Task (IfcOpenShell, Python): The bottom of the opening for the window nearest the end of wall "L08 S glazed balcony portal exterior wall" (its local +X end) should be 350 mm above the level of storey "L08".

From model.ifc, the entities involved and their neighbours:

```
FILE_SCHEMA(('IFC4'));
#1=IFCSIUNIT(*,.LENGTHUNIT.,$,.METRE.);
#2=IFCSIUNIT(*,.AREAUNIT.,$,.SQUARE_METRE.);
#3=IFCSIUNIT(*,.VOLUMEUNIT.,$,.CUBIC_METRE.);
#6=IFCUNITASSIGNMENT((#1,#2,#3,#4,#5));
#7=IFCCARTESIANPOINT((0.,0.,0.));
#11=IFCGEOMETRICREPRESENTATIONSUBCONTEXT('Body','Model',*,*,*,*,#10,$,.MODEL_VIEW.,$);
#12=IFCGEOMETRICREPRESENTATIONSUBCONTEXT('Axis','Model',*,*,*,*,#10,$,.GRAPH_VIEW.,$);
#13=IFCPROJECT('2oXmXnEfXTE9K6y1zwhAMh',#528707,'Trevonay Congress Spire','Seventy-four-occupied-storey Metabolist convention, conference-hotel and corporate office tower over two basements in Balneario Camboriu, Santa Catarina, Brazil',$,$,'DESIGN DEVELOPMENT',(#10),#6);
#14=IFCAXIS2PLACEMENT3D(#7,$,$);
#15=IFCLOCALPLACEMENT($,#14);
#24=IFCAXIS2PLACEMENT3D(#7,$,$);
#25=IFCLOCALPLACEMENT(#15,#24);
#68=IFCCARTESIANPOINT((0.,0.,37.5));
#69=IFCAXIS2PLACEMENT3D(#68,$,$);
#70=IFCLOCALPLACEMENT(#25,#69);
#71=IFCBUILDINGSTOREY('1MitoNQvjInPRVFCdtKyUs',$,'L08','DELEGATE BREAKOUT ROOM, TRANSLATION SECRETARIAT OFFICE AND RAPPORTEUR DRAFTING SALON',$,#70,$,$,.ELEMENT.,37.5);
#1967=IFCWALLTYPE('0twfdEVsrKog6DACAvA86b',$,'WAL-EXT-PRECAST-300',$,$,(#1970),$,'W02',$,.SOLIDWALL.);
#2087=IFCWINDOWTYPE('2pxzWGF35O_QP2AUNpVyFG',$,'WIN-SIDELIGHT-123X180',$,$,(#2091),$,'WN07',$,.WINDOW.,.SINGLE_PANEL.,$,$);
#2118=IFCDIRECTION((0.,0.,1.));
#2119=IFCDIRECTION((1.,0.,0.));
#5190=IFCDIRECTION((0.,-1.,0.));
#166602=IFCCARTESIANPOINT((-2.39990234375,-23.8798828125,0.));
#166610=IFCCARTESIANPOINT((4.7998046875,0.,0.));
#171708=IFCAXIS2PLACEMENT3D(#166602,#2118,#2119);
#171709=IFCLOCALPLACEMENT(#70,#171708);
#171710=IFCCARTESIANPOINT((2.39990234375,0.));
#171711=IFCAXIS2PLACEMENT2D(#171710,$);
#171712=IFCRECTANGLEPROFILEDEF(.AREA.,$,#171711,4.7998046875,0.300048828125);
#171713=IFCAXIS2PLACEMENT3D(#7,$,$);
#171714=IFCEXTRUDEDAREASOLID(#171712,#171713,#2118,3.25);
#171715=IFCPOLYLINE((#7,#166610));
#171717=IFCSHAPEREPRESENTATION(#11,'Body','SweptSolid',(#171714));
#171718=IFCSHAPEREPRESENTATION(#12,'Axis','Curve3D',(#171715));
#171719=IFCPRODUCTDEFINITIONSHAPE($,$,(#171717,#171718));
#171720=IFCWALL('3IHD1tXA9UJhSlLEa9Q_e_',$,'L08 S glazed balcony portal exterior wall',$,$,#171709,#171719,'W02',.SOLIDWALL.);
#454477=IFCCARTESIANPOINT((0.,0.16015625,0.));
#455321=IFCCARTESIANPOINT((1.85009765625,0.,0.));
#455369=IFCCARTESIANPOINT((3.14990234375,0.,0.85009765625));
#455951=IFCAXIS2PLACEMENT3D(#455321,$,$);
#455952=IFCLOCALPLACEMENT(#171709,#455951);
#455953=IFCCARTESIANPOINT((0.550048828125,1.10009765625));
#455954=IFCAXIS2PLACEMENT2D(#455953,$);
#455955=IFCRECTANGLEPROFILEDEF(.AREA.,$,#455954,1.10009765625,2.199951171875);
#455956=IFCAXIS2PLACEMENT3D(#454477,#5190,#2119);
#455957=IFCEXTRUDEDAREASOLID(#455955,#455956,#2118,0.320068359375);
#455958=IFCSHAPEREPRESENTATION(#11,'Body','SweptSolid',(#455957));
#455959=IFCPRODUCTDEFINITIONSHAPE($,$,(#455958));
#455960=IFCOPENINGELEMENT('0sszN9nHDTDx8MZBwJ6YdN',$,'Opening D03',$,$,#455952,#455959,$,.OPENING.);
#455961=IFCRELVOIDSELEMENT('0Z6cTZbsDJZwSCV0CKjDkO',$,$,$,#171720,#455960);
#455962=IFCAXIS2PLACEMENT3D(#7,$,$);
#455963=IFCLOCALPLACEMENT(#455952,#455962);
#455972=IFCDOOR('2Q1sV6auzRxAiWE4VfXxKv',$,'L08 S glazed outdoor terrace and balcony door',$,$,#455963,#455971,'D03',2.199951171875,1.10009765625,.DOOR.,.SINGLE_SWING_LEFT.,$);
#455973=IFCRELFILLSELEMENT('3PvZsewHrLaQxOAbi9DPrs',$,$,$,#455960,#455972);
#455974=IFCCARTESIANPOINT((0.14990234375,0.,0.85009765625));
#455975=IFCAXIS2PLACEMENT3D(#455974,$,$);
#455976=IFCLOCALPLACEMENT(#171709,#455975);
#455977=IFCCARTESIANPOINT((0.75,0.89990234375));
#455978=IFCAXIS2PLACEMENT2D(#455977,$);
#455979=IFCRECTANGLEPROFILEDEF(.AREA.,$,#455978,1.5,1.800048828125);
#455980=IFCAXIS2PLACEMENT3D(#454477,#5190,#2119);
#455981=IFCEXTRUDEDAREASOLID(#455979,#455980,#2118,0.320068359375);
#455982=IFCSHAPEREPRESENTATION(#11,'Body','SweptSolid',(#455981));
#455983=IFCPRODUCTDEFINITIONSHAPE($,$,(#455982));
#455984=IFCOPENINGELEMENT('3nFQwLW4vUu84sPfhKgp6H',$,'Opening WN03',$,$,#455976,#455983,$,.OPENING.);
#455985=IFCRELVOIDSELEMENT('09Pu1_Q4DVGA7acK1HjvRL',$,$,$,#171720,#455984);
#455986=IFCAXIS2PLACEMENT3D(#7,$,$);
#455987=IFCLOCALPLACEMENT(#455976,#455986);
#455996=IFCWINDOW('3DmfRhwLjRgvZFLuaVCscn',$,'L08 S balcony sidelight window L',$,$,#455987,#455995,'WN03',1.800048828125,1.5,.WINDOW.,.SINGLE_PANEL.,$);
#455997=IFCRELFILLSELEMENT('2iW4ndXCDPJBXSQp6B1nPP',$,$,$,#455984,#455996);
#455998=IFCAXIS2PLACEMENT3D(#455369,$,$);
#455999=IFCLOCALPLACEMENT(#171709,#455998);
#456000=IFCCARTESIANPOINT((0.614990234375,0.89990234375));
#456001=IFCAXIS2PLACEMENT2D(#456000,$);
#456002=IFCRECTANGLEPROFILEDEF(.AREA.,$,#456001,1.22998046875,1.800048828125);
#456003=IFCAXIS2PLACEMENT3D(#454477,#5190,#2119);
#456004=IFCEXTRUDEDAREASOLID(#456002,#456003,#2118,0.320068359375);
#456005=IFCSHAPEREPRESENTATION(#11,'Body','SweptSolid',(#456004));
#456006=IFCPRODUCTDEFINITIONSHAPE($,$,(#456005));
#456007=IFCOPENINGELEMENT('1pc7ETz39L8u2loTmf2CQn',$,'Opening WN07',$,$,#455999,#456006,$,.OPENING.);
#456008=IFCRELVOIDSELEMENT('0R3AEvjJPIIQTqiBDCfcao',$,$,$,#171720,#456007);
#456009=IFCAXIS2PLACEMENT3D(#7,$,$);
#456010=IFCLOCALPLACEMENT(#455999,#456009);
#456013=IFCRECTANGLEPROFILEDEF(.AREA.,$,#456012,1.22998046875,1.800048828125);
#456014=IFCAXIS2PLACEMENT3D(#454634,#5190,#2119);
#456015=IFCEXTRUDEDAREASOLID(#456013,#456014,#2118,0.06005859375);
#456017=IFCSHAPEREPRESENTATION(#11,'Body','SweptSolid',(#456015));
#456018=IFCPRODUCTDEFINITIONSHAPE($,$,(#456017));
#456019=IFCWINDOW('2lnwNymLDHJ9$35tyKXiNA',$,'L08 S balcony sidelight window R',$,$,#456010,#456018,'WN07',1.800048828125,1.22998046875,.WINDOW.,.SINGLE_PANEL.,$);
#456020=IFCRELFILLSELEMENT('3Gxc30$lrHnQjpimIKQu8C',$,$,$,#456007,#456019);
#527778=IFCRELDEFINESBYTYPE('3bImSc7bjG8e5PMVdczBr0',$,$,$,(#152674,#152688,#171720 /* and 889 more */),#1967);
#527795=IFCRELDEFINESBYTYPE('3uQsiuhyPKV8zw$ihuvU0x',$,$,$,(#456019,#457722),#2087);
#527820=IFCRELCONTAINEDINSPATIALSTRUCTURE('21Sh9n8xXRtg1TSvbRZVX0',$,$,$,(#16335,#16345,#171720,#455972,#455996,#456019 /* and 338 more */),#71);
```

```python
import numpy as np
import ifcopenshell
import ifcopenshell.api.geometry
import ifcopenshell.geom
import ifcopenshell.util.element
import ifcopenshell.util.placement
import ifcopenshell.util.shape
import ifcopenshell.util.unit

model = ifcopenshell.open("model.ifc")
unit_scale = ifcopenshell.util.unit.calculate_unit_scale(model)

window = model.by_guid("2lnwNymLDHJ9$35tyKXiNA")
opening = window.FillsVoids[0].RelatingOpeningElement
storey = ifcopenshell.util.element.get_container(window, ifc_class="IfcBuildingStorey")
level = ifcopenshell.util.placement.get_local_placement(storey.ObjectPlacement)[2, 3]

# The opening's origin need not be at the sill, so measure its lowest point.
shape = ifcopenshell.geom.create_shape(ifcopenshell.geom.settings(), opening)
bottom = ifcopenshell.util.shape.get_shape_bottom_elevation(shape, shape.geometry) / unit_scale
dz = level + 0.35 / unit_scale - bottom

shift = np.array([0.0, 0.0, dz])
# The window is placed relative to its opening, so it follows when the opening moves.
matrix = ifcopenshell.util.placement.get_local_placement(opening.ObjectPlacement)
matrix[:3, 3] += shift
ifcopenshell.api.geometry.edit_object_placement(
    model, product=opening, matrix=matrix, is_si=False, should_transform_children=True
)

print(f"moved by {dz * unit_scale:+.3f} m")

model.write("model_rev.ifc")
```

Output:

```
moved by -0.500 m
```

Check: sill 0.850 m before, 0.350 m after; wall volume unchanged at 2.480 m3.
